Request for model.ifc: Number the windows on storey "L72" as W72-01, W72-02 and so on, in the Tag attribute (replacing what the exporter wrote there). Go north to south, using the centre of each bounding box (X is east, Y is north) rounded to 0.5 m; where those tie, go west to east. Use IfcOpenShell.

First a look at what the model holds.

```python
import ifcopenshell
import ifcopenshell.util.element
import ifcopenshell.util.placement

model = ifcopenshell.open("model.ifc")
print(model.schema)
storey = next(s for s in model.by_type("IfcBuildingStorey") if s.Name == "L72")
windows = [e for e in ifcopenshell.util.element.get_decomposition(storey) if e.is_a("IfcWindow")]
for e in sorted(windows, key=lambda e: e.id()):
    origin = ifcopenshell.util.placement.get_local_placement(e.ObjectPlacement)[:3, 3]
    print(e.id(), e.Tag, e.Name, origin.round(2) + 0.0, sep=" | ")
```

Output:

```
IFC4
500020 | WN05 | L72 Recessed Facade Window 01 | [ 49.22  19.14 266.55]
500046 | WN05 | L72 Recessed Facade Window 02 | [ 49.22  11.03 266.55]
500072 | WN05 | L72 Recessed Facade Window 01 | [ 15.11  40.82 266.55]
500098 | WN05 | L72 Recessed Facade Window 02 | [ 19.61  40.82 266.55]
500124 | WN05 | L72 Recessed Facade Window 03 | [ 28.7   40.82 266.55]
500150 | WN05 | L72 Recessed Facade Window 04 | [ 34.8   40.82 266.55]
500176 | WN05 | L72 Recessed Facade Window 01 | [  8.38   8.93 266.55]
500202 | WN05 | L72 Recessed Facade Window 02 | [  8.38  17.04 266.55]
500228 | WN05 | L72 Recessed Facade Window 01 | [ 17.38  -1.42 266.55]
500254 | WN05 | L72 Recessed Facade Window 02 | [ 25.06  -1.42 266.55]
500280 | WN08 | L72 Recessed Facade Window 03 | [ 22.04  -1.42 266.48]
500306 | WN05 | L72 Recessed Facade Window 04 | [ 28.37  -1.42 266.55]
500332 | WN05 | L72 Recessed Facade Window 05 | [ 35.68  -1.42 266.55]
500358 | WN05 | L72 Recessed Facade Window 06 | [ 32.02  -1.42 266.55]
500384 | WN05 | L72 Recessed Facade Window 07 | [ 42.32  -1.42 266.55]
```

```python
import ifcopenshell
import ifcopenshell.geom
import ifcopenshell.util.element
import ifcopenshell.util.shape

model = ifcopenshell.open("model.ifc")
settings = ifcopenshell.geom.settings()
settings.set("use-world-coords", True)


def centre(element):
    shape = ifcopenshell.geom.create_shape(settings, element)
    return ifcopenshell.util.shape.get_bbox_centroid(shape.geometry)


storey = next(s for s in model.by_type("IfcBuildingStorey") if s.Name == "L72")
windows = [e for e in ifcopenshell.util.element.get_decomposition(storey) if e.is_a("IfcWindow")]

# Insertion points can sit at a corner or the storey origin, so sort by the geometry (in metres).
centres = {e: centre(e) for e in windows}
windows.sort(key=lambda e: (-round(centres[e][1] / 0.5), centres[e][0]))

for i, e in enumerate(windows, start=1):
    number = f"W72-{i:02d}"
    e.Tag = number
    print(e.id(), number)

model.write("model_rev.ifc")
```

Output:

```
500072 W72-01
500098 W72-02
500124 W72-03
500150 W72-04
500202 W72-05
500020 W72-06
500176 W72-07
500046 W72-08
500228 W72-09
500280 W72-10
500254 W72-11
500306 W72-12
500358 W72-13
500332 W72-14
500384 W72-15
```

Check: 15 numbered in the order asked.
